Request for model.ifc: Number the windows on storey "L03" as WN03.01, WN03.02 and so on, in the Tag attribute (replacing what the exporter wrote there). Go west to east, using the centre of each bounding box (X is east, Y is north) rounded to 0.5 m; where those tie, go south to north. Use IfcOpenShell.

First a look at what the model holds.

```python
import ifcopenshell
import ifcopenshell.util.element
import ifcopenshell.util.placement

model = ifcopenshell.open("model.ifc")
print(model.schema)
storey = next(s for s in model.by_type("IfcBuildingStorey") if s.Name == "L03")
windows = [e for e in ifcopenshell.util.element.get_decomposition(storey) if e.is_a("IfcWindow")]
for e in sorted(windows, key=lambda e: e.id()):
    origin = ifcopenshell.util.placement.get_local_placement(e.ObjectPlacement)[:3, 3]
    print(e.id(), e.Tag, e.Name, origin.round(2) + 0.0, sep=" | ")
```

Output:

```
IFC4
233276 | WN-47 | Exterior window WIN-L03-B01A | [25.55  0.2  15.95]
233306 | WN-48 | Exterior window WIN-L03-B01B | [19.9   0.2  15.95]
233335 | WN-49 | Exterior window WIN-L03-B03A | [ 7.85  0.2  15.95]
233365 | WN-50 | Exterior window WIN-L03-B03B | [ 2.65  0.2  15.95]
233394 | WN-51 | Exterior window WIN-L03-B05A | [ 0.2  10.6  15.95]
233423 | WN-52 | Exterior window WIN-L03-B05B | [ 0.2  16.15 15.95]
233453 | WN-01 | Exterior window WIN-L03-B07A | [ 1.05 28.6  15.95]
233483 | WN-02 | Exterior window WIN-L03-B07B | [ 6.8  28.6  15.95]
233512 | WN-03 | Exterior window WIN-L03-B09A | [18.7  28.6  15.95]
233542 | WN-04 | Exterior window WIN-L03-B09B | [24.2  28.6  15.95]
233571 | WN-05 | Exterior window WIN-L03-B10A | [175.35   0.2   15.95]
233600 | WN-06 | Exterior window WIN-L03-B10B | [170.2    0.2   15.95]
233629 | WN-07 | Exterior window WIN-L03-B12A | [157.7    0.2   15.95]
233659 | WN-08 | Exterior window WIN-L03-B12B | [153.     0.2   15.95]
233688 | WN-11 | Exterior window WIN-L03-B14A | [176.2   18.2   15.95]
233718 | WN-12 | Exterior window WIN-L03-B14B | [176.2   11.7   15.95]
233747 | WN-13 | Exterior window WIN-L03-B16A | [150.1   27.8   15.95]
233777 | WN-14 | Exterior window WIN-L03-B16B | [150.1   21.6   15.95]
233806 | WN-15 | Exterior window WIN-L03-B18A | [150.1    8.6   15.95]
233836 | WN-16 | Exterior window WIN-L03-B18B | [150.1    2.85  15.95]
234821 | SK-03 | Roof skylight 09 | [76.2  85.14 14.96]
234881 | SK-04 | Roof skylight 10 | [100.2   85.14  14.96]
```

```python
import ifcopenshell
import ifcopenshell.geom
import ifcopenshell.util.element
import ifcopenshell.util.shape

model = ifcopenshell.open("model.ifc")
settings = ifcopenshell.geom.settings()
settings.set("use-world-coords", True)


def centre(element):
    shape = ifcopenshell.geom.create_shape(settings, element)
    return ifcopenshell.util.shape.get_bbox_centroid(shape.geometry)


storey = next(s for s in model.by_type("IfcBuildingStorey") if s.Name == "L03")
windows = [e for e in ifcopenshell.util.element.get_decomposition(storey) if e.is_a("IfcWindow")]

# Insertion points can sit at a corner or the storey origin, so sort by the geometry (in metres).
centres = {e: centre(e) for e in windows}
windows.sort(key=lambda e: (round(centres[e][0] / 0.5), centres[e][1]))

for i, e in enumerate(windows, start=1):
    number = f"WN03.{i:02d}"
    e.Tag = number
    print(e.id(), number)

model.write("model_edited.ifc")
```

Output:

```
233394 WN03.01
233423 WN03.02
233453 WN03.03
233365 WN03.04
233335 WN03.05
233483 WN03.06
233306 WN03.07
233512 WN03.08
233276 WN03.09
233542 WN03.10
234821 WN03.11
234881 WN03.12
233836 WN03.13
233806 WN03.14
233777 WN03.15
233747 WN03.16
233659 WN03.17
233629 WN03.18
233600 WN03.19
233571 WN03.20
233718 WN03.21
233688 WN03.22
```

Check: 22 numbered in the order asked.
